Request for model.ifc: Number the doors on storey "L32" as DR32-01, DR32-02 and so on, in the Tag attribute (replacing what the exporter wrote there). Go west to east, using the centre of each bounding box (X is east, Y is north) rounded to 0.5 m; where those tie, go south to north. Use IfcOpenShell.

First a look at what the model holds.

```python
import ifcopenshell
import ifcopenshell.util.element
import ifcopenshell.util.placement

model = ifcopenshell.open("model.ifc")
print(model.schema)
storey = next(s for s in model.by_type("IfcBuildingStorey") if s.Name == "L32")
doors = [e for e in ifcopenshell.util.element.get_decomposition(storey) if e.is_a("IfcDoor")]
for e in sorted(doors, key=lambda e: e.id()):
    origin = ifcopenshell.util.placement.get_local_placement(e.ObjectPlacement)[:3, 3]
    print(e.id(), e.Tag, e.Name, origin.round(2) + 0.0, sep=" | ")
```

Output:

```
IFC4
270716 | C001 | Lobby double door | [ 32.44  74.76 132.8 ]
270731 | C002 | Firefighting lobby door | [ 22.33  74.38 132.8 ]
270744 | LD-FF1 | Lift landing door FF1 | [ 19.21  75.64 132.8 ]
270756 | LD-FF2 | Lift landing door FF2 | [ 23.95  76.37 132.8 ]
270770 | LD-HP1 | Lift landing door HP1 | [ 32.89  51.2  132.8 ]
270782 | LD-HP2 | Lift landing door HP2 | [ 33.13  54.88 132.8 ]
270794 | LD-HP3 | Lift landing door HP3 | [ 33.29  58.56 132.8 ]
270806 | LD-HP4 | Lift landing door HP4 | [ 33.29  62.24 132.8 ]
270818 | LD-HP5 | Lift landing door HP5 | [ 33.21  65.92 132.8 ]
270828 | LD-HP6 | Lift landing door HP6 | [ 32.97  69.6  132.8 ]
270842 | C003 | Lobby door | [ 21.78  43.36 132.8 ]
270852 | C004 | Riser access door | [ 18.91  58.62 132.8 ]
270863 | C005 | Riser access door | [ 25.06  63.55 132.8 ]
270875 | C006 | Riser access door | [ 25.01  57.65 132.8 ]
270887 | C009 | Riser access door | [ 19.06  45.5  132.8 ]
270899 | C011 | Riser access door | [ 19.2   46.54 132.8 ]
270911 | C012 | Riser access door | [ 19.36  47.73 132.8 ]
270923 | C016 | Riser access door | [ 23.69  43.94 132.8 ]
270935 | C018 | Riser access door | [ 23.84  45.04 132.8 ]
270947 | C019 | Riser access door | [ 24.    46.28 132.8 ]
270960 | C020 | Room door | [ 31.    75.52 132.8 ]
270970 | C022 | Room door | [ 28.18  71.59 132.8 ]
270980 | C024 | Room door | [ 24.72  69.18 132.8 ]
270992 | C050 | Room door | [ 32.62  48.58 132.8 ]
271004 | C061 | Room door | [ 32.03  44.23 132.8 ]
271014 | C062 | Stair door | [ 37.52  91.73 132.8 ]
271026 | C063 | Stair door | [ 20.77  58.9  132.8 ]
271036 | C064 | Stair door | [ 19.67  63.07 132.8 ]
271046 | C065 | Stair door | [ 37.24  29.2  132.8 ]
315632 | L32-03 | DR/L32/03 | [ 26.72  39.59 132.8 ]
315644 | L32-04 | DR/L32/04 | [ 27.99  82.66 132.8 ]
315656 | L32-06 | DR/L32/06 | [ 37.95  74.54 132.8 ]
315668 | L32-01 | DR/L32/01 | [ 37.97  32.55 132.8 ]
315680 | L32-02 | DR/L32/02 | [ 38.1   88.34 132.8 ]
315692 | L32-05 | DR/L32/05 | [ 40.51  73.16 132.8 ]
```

```python
import ifcopenshell
import ifcopenshell.geom
import ifcopenshell.util.element
import ifcopenshell.util.shape

model = ifcopenshell.open("model.ifc")
settings = ifcopenshell.geom.settings()
settings.set("use-world-coords", True)


def centre(element):
    shape = ifcopenshell.geom.create_shape(settings, element)
    return ifcopenshell.util.shape.get_bbox_centroid(shape.geometry)


storey = next(s for s in model.by_type("IfcBuildingStorey") if s.Name == "L32")
doors = [e for e in ifcopenshell.util.element.get_decomposition(storey) if e.is_a("IfcDoor")]

# Insertion points can sit at a corner or the storey origin, so sort by the geometry (in metres).
centres = {e: centre(e) for e in doors}
doors.sort(key=lambda e: (round(centres[e][0] / 0.5), centres[e][1]))

for i, e in enumerate(doors, start=1):
    number = f"DR32-{i:02d}"
    e.Tag = number
    print(e.id(), number)

model.write("model-out.ifc")
```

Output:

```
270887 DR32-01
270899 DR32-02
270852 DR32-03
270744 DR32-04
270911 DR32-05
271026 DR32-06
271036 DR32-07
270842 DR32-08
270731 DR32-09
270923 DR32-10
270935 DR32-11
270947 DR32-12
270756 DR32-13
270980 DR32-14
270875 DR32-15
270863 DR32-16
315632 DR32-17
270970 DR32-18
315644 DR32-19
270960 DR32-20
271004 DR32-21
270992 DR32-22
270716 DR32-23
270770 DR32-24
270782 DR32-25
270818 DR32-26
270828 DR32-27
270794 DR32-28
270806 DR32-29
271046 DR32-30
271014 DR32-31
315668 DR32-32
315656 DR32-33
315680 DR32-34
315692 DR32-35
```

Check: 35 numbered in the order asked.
